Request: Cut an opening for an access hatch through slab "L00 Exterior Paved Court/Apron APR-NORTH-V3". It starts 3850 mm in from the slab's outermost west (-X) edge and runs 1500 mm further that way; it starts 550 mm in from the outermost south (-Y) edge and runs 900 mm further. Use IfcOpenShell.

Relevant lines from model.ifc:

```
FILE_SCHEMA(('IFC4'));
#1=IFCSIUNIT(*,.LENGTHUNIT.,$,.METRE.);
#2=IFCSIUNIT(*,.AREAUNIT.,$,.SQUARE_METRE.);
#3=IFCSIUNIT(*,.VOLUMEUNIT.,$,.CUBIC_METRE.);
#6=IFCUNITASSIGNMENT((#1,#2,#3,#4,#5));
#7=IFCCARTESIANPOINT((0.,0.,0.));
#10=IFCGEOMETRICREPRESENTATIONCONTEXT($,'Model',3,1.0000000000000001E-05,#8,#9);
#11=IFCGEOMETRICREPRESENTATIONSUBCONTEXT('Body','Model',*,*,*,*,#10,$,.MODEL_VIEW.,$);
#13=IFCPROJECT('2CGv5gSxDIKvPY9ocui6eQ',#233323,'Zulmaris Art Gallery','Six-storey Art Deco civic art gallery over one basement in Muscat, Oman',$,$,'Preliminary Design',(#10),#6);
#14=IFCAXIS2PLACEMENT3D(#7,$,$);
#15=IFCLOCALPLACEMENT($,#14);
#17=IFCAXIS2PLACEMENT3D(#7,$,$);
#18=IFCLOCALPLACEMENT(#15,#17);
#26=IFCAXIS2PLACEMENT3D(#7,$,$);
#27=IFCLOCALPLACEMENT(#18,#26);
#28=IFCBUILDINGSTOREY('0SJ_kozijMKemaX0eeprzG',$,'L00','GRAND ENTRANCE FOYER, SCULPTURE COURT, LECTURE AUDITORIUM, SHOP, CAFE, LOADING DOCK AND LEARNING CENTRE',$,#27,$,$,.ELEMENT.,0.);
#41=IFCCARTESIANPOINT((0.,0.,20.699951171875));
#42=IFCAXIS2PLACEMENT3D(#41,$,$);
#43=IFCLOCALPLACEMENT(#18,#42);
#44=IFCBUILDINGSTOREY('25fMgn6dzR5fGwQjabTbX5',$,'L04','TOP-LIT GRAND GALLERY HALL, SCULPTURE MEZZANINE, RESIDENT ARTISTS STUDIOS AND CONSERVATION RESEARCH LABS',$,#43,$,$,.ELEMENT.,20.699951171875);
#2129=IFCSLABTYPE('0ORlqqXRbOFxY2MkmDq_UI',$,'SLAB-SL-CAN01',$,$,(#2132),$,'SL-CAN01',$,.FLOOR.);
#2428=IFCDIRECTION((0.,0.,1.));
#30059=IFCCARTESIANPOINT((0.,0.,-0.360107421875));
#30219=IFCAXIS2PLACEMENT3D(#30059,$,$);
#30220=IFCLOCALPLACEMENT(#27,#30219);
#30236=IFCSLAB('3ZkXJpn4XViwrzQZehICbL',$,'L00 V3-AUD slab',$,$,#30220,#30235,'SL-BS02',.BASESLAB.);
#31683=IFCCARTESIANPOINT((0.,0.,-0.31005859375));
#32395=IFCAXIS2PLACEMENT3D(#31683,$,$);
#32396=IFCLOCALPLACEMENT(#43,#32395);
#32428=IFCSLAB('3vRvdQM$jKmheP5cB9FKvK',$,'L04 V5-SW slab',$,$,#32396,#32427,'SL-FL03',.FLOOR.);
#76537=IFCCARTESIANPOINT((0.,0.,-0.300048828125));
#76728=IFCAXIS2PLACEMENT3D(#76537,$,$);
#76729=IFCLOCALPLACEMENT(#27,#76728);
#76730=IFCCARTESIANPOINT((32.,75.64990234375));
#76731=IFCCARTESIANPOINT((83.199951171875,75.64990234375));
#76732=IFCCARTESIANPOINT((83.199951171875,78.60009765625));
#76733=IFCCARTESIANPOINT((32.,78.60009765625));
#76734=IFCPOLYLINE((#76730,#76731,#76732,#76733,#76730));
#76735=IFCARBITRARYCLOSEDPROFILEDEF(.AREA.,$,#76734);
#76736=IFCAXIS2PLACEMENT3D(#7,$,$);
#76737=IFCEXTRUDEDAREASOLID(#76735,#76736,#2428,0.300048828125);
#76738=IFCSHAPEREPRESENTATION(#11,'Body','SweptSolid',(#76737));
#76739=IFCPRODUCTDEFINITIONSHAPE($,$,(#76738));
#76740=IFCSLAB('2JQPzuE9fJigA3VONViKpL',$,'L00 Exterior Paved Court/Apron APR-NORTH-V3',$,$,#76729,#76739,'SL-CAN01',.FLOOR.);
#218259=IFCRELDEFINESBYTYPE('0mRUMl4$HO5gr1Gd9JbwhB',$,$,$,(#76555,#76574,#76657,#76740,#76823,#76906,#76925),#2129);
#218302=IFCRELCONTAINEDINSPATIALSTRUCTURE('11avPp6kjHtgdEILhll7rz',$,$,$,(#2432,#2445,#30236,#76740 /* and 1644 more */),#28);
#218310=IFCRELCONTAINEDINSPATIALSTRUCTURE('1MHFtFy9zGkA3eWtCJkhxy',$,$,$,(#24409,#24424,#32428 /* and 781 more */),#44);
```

```python
import numpy as np
import ifcopenshell
import ifcopenshell.api.feature
import ifcopenshell.api.geometry
import ifcopenshell.api.root
import ifcopenshell.geom
import ifcopenshell.util.placement
import ifcopenshell.util.representation
import ifcopenshell.util.shape
import ifcopenshell.util.unit

model = ifcopenshell.open("model.ifc")
unit_scale = ifcopenshell.util.unit.calculate_unit_scale(model)
settings = ifcopenshell.geom.settings()


def volume(element):
    """Net volume in cubic metres, openings subtracted."""
    shape = ifcopenshell.geom.create_shape(settings, element)
    return ifcopenshell.util.shape.get_volume(shape.geometry)


slab = model.by_id(76740)
before = volume(slab)

# Extent in the slab's own axes, in metres. The edges named are its -X and -Y sides.
slab_shape = ifcopenshell.geom.create_shape(settings, slab)
vertices = ifcopenshell.util.shape.get_vertices(slab_shape.geometry)
x_min, y_min, bottom = vertices.min(axis=0)
top = vertices[:, 2].max()

opening = ifcopenshell.api.root.create_entity(model, ifc_class="IfcOpeningElement", name="Access hatch opening", predefined_type="OPENING")
context = ifcopenshell.util.representation.get_context(model, "Model", "Body", "MODEL_VIEW")
width, depth = 1.5, 0.9
outline = [(0.0, 0.0), (width, 0.0), (width, depth), (0.0, depth), (0.0, 0.0)]
# Overshoot both faces by 50 mm so the cut is clean.
shape = ifcopenshell.api.geometry.add_slab_representation(
    model, context=context, depth=top - bottom + 0.1, polyline=outline
)
ifcopenshell.api.geometry.assign_representation(model, product=opening, representation=shape)

matrix = ifcopenshell.util.placement.get_local_placement(slab.ObjectPlacement)
matrix[:, 3] = matrix @ np.append(np.array([x_min + 3.85, y_min + 0.55, bottom - 0.05]) / unit_scale, 1.0)
ifcopenshell.api.geometry.edit_object_placement(model, product=opening, matrix=matrix, is_si=False)
ifcopenshell.api.feature.add_feature(model, feature=opening, element=slab)

after = volume(slab)

print(f"slab volume {before:.3f} -> {after:.3f} m3")

model.write("model_edited.ifc")
```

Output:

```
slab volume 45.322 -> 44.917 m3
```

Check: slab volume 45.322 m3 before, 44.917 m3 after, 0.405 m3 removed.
